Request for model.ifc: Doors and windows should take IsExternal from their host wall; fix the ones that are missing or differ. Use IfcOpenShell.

First a look at what the model holds.

```python
import ifcopenshell
import ifcopenshell.util.element

model = ifcopenshell.open("model.ifc")
print(model.schema)
seen = {}
for e in model.by_type("IfcDoor") + model.by_type("IfcWindow"):
    if not e.FillsVoids:
        continue
    host = e.FillsVoids[0].RelatingOpeningElement.VoidsElements[0].RelatingBuildingElement
    own = ifcopenshell.util.element.get_pset(e, f"Pset_{e.is_a()[3:].removesuffix('StandardCase')}Common", "IsExternal")
    wall = ifcopenshell.util.element.get_pset(host, "Pset_WallCommon", "IsExternal")
    seen[e.is_a(), own, wall] = seen.get((e.is_a(), own, wall), 0) + 1
for (cls, own, wall), count in sorted(seen.items(), key=str):
    print(count, cls, "IsExternal:", own, "| host wall:", wall)
```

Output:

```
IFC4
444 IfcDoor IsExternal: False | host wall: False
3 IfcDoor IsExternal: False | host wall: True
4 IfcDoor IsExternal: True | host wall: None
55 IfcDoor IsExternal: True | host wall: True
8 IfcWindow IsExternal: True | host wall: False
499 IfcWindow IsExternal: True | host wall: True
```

```python
import ifcopenshell
import ifcopenshell.api.pset
import ifcopenshell.util.element

model = ifcopenshell.open("model.ifc")

count = 0
for ifc_class, pset_name in (("IfcDoor", "Pset_DoorCommon"), ("IfcWindow", "Pset_WindowCommon")):
    for e in model.by_type(ifc_class):
        if not e.FillsVoids:
            continue
        host = e.FillsVoids[0].RelatingOpeningElement.VoidsElements[0].RelatingBuildingElement
        external = ifcopenshell.util.element.get_pset(host, "Pset_WallCommon", "IsExternal")
        if external is None or ifcopenshell.util.element.get_pset(e, pset_name, "IsExternal") == external:
            continue
        pset = ifcopenshell.api.pset.add_pset(model, product=e, name=pset_name)
        ifcopenshell.api.pset.edit_pset(model, pset=pset, properties={"IsExternal": external})
        count += 1

print(count, "updated")

model.write("model-out.ifc")
```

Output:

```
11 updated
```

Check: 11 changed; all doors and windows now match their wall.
